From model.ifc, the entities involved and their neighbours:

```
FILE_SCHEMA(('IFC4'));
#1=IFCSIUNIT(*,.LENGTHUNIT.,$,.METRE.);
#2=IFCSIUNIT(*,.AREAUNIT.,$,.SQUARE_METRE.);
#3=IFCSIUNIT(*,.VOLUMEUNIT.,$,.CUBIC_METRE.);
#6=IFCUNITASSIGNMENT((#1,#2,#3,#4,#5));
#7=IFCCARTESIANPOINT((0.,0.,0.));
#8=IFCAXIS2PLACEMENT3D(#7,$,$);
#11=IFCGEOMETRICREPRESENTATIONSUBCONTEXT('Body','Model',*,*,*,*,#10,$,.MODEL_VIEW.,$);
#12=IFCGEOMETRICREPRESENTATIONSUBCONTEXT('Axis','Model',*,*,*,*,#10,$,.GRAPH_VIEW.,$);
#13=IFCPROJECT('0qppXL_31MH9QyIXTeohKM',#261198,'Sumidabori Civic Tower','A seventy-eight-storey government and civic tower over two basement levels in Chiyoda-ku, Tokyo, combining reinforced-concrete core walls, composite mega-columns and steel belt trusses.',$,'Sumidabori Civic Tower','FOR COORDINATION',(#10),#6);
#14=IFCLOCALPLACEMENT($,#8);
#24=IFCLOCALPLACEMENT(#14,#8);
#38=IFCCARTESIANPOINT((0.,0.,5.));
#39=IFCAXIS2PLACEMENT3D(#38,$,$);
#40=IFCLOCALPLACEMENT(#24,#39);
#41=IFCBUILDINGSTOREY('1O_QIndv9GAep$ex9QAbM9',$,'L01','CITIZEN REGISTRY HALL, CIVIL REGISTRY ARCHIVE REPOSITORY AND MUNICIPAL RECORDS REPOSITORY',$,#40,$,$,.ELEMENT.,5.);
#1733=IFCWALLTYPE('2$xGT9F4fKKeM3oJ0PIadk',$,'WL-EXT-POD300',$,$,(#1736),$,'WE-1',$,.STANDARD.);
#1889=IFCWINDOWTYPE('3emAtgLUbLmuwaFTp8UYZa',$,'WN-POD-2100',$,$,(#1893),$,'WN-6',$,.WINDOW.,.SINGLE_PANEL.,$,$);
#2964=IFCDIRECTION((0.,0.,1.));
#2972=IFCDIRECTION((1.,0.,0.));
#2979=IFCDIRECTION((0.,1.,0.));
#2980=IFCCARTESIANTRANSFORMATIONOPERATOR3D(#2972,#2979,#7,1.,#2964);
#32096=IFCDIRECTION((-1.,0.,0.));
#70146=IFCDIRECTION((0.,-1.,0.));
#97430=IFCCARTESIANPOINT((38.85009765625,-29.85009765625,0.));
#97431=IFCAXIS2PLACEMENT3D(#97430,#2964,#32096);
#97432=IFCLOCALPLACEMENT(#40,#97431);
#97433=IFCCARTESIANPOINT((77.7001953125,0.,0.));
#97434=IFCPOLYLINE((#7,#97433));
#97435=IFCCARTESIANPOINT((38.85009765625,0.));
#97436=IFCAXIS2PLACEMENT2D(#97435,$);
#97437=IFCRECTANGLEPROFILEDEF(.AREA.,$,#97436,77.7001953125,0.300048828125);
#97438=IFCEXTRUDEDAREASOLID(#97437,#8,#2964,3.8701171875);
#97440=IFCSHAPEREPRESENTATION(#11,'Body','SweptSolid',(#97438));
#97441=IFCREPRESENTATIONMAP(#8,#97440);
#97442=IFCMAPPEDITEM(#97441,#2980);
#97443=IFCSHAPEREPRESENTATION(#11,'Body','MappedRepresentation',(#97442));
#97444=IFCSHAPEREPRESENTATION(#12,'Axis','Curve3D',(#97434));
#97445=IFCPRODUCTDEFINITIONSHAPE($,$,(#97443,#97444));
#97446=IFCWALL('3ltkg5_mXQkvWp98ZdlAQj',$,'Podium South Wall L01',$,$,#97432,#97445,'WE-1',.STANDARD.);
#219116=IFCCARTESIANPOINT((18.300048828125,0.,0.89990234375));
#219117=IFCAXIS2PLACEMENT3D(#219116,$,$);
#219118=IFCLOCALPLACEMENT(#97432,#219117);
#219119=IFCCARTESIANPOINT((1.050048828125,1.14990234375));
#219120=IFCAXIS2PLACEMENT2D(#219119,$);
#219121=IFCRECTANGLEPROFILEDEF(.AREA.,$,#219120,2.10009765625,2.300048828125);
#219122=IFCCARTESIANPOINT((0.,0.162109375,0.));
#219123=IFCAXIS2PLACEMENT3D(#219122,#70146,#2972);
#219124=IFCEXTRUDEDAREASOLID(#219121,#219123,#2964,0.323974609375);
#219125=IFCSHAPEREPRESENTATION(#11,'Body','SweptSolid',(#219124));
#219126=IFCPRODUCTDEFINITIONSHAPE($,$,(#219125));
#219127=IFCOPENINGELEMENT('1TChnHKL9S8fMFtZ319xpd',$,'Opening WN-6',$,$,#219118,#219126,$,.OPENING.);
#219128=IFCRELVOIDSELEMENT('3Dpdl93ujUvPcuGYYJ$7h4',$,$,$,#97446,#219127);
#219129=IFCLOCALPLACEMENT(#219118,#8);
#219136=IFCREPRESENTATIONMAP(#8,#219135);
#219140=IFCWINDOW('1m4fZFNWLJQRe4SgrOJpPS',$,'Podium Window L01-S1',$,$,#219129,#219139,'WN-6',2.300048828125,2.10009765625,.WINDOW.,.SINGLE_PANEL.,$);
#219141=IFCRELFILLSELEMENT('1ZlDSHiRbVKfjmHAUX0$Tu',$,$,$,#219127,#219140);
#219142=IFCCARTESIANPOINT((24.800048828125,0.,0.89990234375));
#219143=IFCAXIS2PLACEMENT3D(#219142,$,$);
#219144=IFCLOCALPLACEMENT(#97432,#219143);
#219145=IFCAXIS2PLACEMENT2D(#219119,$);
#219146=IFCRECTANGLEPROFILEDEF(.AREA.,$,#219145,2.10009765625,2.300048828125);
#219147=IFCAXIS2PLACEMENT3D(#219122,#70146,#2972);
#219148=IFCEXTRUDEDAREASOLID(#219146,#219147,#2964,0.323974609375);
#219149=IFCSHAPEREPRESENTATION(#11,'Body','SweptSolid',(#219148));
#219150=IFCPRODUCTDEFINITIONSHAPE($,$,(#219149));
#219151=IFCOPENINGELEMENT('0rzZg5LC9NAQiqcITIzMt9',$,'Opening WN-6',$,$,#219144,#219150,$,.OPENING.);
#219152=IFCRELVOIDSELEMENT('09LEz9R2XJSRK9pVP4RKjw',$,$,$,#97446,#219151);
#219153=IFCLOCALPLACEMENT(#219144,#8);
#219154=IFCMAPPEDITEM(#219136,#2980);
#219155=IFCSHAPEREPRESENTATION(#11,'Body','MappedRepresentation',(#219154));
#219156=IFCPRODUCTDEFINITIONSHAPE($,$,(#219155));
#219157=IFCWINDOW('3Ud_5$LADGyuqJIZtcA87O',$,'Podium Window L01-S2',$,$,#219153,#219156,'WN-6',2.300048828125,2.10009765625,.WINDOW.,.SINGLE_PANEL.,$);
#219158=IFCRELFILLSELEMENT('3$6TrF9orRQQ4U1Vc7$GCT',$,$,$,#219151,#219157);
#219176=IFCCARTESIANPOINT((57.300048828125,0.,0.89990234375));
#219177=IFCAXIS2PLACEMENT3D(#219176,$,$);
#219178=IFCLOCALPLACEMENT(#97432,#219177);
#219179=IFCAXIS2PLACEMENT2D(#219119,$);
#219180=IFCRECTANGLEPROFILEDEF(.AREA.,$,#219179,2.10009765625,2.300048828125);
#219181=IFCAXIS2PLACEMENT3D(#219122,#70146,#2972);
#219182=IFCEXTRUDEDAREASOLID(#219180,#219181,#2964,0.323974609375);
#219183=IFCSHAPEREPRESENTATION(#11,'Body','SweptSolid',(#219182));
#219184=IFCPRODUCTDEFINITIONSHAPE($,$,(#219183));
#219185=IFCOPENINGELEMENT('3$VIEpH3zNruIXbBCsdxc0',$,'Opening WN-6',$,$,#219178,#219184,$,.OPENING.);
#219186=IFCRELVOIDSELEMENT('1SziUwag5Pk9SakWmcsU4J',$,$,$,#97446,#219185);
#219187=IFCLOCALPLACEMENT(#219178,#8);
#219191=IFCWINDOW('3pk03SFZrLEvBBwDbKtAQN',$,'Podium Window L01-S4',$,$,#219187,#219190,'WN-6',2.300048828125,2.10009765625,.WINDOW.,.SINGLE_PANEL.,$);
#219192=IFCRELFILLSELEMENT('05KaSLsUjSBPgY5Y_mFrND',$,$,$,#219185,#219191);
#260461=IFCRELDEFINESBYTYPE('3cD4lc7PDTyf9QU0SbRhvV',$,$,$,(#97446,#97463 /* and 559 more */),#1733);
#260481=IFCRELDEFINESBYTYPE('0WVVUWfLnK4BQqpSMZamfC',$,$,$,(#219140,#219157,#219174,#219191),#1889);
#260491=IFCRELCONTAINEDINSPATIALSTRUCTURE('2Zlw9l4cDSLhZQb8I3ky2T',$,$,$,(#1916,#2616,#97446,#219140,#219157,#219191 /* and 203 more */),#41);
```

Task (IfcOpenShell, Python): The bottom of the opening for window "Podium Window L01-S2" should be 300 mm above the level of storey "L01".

```python
import numpy as np
import ifcopenshell
import ifcopenshell.api.geometry
import ifcopenshell.geom
import ifcopenshell.util.element
import ifcopenshell.util.placement
import ifcopenshell.util.shape
import ifcopenshell.util.unit

model = ifcopenshell.open("model.ifc")
unit_scale = ifcopenshell.util.unit.calculate_unit_scale(model)

window = model.by_guid("3Ud_5$LADGyuqJIZtcA87O")
opening = window.FillsVoids[0].RelatingOpeningElement
storey = ifcopenshell.util.element.get_container(window, ifc_class="IfcBuildingStorey")
level = ifcopenshell.util.placement.get_local_placement(storey.ObjectPlacement)[2, 3]

# The opening's origin need not be at the sill, so measure its lowest point.
shape = ifcopenshell.geom.create_shape(ifcopenshell.geom.settings(), opening)
bottom = ifcopenshell.util.shape.get_shape_bottom_elevation(shape, shape.geometry) / unit_scale
dz = level + 0.3 - bottom

shift = np.array([0.0, 0.0, dz])
# The window is placed relative to its opening, so it follows when the opening moves.
matrix = ifcopenshell.util.placement.get_local_placement(opening.ObjectPlacement)
matrix[:3, 3] += shift
ifcopenshell.api.geometry.edit_object_placement(
    model, product=opening, matrix=matrix, is_si=False, should_transform_children=True
)

print(f"moved by {dz * unit_scale:+.3f} m")

model.write("model_edited.ifc")
```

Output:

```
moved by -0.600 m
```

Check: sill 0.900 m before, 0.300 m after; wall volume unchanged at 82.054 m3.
